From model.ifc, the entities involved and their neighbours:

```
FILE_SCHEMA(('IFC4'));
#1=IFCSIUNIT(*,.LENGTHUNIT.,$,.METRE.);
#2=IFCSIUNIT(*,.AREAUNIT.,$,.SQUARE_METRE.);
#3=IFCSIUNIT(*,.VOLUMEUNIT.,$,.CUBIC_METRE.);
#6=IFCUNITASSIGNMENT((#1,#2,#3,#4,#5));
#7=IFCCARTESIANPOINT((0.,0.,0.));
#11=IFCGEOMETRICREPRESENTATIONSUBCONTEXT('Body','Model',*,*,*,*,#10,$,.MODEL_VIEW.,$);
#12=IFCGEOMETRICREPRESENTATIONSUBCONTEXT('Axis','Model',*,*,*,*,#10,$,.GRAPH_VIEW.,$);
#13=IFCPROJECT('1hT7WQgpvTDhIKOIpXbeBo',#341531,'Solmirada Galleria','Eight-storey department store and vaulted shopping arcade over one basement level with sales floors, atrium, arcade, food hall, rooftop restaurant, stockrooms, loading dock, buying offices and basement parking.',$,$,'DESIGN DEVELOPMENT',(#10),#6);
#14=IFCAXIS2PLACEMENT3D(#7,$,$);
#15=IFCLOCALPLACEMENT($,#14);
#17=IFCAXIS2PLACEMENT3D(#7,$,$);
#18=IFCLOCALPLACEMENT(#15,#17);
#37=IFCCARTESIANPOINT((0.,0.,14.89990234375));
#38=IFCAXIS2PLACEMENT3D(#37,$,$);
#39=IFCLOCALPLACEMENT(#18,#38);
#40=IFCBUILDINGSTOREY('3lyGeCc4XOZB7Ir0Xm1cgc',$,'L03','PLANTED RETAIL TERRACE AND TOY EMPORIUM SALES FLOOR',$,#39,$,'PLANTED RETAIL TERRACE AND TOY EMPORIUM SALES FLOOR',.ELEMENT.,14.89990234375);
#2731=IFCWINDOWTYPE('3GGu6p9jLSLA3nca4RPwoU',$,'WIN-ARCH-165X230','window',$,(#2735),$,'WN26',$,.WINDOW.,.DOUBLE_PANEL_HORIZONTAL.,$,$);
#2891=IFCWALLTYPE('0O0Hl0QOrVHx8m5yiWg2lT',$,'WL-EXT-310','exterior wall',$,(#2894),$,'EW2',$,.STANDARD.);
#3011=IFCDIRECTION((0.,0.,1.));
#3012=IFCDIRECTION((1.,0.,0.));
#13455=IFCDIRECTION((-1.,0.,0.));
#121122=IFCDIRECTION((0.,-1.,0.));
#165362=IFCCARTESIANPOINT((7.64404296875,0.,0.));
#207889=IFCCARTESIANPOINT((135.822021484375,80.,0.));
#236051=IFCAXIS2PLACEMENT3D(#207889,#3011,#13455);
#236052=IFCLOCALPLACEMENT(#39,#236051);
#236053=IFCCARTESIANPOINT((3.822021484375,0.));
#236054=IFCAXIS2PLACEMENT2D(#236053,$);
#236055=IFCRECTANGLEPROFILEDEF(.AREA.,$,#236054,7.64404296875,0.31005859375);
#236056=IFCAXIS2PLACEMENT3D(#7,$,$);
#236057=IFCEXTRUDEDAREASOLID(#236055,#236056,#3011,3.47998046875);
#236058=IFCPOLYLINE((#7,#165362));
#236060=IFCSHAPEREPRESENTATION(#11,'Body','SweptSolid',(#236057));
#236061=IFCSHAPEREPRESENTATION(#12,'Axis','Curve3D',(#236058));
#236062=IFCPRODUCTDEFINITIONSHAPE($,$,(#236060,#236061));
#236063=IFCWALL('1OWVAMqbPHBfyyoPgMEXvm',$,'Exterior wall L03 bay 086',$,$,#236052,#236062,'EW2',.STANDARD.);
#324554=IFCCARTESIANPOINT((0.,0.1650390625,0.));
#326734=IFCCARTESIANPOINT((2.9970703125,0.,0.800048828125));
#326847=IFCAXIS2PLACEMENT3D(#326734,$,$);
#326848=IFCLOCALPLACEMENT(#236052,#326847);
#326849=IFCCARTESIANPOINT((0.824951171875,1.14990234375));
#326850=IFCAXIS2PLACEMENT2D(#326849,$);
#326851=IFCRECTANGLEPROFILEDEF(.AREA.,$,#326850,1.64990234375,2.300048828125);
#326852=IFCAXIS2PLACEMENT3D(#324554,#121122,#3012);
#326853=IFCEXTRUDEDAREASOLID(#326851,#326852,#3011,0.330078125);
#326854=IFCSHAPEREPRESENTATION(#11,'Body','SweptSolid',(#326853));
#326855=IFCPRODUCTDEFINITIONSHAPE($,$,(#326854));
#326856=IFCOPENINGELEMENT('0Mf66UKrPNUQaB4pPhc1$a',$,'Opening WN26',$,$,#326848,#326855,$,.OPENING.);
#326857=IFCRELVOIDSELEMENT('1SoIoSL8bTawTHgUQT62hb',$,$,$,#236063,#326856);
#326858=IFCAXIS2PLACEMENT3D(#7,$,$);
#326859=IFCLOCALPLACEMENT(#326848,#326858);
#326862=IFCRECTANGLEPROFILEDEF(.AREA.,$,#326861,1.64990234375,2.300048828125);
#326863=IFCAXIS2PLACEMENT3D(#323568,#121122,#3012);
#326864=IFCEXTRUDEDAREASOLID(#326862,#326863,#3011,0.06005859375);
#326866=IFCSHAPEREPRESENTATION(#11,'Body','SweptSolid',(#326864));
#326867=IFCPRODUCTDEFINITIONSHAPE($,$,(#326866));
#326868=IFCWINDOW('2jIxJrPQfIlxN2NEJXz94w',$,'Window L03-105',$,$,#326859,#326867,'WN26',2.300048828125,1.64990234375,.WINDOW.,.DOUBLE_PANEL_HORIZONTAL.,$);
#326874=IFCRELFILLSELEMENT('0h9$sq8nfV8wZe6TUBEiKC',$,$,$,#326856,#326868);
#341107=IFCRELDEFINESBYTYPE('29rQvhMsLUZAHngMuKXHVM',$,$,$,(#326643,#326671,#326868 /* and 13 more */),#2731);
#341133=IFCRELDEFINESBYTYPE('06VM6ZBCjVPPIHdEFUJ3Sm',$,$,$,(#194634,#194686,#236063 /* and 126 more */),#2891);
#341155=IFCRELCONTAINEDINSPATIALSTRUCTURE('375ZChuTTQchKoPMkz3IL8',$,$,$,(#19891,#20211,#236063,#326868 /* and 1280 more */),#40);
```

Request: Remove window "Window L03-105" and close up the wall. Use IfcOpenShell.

```python
import ifcopenshell
import ifcopenshell.api.feature
import ifcopenshell.api.root
import ifcopenshell.geom
import ifcopenshell.util.shape

model = ifcopenshell.open("model.ifc")
settings = ifcopenshell.geom.settings()


def volume(element):
    """Net volume in cubic metres, openings subtracted."""
    shape = ifcopenshell.geom.create_shape(settings, element)
    return ifcopenshell.util.shape.get_volume(shape.geometry)


window = model.by_guid("2jIxJrPQfIlxN2NEJXz94w")
opening = window.FillsVoids[0].RelatingOpeningElement
wall = opening.VoidsElements[0].RelatingBuildingElement
before = volume(wall)

ifcopenshell.api.root.remove_product(model, product=window)
ifcopenshell.api.feature.remove_feature(model, feature=opening)

after = volume(wall)

print(f"wall volume {before:.3f} -> {after:.3f} m3")

model.write("model_edited.ifc")
```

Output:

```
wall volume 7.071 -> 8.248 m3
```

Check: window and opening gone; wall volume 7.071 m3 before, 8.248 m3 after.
